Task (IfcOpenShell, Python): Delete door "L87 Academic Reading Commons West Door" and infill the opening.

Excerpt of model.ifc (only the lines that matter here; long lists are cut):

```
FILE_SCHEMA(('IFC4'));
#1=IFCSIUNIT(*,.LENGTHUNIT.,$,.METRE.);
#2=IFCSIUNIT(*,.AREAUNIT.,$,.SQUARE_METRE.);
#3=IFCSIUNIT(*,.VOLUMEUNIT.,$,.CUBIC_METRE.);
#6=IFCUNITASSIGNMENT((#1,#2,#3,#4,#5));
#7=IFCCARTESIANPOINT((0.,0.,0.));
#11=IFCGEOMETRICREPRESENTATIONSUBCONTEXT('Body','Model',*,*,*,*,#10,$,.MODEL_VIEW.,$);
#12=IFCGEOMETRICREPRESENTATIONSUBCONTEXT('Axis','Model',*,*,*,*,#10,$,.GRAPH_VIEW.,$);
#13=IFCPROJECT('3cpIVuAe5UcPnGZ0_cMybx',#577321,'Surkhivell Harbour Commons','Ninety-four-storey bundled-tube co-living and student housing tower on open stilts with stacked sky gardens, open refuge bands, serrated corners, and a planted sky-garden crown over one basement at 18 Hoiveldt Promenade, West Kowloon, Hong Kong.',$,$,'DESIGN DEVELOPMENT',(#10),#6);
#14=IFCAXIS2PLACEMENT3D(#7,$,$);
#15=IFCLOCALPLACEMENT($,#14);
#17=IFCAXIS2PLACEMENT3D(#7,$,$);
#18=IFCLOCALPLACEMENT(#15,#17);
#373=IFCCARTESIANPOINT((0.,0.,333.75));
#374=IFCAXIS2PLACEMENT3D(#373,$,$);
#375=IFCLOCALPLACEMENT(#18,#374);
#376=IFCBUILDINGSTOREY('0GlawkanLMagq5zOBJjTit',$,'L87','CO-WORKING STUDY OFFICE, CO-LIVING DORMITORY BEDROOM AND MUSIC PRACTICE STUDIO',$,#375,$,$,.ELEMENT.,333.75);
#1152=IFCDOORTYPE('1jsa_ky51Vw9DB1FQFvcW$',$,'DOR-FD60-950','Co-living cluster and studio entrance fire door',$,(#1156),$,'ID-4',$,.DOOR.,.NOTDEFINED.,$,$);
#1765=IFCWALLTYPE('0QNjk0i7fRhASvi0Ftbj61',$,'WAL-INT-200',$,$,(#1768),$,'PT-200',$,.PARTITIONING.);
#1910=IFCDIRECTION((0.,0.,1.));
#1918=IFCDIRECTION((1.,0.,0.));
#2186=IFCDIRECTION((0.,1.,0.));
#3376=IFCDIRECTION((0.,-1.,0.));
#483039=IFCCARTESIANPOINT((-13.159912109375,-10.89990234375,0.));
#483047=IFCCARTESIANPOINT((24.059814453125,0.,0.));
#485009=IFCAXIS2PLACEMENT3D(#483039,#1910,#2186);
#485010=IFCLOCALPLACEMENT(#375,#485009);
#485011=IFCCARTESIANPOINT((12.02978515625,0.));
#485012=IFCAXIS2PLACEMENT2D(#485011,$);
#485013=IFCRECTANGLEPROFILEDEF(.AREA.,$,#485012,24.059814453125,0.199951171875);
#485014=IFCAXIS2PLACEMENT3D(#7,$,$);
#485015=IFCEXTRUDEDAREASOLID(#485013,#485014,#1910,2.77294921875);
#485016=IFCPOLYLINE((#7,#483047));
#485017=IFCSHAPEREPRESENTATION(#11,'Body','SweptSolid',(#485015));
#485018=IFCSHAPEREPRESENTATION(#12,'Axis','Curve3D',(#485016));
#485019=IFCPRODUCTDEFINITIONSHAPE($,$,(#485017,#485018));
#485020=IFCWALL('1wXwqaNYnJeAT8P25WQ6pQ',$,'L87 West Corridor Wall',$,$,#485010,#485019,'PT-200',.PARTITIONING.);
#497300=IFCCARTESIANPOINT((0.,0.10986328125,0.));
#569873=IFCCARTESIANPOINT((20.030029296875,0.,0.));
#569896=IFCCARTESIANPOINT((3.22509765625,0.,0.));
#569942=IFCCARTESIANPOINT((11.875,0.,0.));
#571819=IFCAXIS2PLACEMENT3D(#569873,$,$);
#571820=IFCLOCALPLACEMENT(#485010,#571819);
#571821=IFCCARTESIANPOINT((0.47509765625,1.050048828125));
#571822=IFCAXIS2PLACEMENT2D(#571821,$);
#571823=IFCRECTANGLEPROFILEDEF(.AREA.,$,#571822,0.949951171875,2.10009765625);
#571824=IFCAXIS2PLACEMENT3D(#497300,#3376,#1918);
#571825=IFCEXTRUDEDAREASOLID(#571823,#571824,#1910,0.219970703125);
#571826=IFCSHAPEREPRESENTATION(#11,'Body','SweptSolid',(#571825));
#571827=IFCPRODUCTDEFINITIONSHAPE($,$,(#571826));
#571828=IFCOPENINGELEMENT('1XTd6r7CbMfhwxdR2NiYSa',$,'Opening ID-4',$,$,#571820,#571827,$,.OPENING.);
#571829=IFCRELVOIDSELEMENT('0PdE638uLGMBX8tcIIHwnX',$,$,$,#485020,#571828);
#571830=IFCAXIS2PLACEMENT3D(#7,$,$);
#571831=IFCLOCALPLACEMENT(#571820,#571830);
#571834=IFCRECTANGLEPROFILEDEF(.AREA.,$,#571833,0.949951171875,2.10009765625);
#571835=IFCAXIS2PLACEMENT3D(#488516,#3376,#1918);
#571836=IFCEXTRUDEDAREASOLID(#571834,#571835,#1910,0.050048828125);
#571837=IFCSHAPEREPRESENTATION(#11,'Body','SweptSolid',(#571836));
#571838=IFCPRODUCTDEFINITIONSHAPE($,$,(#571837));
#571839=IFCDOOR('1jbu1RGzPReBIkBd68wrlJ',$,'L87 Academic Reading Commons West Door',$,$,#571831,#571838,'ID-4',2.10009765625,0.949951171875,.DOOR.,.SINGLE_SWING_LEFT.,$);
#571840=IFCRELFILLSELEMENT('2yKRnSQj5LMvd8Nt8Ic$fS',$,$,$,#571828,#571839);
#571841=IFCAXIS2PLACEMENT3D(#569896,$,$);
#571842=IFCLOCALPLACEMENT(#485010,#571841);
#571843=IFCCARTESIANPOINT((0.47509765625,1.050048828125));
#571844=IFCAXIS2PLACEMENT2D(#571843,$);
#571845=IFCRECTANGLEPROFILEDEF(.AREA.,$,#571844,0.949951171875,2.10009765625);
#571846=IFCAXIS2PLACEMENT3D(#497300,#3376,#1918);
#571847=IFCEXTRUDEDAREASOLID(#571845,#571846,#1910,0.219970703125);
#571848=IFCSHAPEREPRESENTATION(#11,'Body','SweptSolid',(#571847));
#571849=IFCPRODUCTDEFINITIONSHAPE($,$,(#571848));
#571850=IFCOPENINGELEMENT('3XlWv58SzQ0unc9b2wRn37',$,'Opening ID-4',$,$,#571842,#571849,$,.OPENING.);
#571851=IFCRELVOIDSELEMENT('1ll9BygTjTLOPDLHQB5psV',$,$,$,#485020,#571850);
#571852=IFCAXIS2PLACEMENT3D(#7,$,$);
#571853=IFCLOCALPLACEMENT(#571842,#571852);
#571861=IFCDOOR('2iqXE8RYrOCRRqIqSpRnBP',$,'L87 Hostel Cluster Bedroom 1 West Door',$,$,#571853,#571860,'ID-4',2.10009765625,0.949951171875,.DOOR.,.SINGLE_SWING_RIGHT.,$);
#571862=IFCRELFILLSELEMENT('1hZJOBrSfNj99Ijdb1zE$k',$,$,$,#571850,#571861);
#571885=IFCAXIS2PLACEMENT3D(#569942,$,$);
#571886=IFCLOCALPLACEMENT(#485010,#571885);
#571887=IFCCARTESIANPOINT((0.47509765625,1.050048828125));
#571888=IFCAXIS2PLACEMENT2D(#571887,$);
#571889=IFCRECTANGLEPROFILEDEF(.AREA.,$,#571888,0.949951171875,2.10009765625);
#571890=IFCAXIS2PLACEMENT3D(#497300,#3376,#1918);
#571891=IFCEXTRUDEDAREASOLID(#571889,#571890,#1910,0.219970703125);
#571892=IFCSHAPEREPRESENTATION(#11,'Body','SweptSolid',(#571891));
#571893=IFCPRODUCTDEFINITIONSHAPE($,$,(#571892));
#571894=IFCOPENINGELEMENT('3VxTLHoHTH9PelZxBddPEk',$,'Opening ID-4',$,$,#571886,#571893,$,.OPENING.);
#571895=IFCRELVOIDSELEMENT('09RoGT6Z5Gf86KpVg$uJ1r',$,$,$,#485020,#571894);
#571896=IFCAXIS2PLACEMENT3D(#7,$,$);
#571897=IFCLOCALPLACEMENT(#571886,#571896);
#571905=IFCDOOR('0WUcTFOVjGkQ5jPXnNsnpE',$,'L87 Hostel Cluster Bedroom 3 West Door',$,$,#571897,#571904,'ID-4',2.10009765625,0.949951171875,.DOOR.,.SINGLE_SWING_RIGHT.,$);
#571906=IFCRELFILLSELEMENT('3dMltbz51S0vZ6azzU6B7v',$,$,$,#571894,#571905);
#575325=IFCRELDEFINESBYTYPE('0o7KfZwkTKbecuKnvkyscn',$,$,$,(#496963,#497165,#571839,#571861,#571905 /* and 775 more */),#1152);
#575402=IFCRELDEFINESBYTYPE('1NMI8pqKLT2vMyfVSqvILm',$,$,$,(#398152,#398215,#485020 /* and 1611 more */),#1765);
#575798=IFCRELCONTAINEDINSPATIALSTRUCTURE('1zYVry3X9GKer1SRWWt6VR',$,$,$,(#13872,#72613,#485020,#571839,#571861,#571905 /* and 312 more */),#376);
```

```python
import ifcopenshell
import ifcopenshell.api.feature
import ifcopenshell.api.root
import ifcopenshell.geom
import ifcopenshell.util.shape

model = ifcopenshell.open("model.ifc")
settings = ifcopenshell.geom.settings()


def volume(element):
    """Net volume in cubic metres, openings subtracted."""
    shape = ifcopenshell.geom.create_shape(settings, element)
    return ifcopenshell.util.shape.get_volume(shape.geometry)


door = model.by_guid("1jbu1RGzPReBIkBd68wrlJ")
opening = door.FillsVoids[0].RelatingOpeningElement
wall = opening.VoidsElements[0].RelatingBuildingElement
before = volume(wall)

ifcopenshell.api.root.remove_product(model, product=door)
ifcopenshell.api.feature.remove_feature(model, feature=opening)

after = volume(wall)

print(f"wall volume {before:.3f} -> {after:.3f} m3")

model.write("model-out.ifc")
```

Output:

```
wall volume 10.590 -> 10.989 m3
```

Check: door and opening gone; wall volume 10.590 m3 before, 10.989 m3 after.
